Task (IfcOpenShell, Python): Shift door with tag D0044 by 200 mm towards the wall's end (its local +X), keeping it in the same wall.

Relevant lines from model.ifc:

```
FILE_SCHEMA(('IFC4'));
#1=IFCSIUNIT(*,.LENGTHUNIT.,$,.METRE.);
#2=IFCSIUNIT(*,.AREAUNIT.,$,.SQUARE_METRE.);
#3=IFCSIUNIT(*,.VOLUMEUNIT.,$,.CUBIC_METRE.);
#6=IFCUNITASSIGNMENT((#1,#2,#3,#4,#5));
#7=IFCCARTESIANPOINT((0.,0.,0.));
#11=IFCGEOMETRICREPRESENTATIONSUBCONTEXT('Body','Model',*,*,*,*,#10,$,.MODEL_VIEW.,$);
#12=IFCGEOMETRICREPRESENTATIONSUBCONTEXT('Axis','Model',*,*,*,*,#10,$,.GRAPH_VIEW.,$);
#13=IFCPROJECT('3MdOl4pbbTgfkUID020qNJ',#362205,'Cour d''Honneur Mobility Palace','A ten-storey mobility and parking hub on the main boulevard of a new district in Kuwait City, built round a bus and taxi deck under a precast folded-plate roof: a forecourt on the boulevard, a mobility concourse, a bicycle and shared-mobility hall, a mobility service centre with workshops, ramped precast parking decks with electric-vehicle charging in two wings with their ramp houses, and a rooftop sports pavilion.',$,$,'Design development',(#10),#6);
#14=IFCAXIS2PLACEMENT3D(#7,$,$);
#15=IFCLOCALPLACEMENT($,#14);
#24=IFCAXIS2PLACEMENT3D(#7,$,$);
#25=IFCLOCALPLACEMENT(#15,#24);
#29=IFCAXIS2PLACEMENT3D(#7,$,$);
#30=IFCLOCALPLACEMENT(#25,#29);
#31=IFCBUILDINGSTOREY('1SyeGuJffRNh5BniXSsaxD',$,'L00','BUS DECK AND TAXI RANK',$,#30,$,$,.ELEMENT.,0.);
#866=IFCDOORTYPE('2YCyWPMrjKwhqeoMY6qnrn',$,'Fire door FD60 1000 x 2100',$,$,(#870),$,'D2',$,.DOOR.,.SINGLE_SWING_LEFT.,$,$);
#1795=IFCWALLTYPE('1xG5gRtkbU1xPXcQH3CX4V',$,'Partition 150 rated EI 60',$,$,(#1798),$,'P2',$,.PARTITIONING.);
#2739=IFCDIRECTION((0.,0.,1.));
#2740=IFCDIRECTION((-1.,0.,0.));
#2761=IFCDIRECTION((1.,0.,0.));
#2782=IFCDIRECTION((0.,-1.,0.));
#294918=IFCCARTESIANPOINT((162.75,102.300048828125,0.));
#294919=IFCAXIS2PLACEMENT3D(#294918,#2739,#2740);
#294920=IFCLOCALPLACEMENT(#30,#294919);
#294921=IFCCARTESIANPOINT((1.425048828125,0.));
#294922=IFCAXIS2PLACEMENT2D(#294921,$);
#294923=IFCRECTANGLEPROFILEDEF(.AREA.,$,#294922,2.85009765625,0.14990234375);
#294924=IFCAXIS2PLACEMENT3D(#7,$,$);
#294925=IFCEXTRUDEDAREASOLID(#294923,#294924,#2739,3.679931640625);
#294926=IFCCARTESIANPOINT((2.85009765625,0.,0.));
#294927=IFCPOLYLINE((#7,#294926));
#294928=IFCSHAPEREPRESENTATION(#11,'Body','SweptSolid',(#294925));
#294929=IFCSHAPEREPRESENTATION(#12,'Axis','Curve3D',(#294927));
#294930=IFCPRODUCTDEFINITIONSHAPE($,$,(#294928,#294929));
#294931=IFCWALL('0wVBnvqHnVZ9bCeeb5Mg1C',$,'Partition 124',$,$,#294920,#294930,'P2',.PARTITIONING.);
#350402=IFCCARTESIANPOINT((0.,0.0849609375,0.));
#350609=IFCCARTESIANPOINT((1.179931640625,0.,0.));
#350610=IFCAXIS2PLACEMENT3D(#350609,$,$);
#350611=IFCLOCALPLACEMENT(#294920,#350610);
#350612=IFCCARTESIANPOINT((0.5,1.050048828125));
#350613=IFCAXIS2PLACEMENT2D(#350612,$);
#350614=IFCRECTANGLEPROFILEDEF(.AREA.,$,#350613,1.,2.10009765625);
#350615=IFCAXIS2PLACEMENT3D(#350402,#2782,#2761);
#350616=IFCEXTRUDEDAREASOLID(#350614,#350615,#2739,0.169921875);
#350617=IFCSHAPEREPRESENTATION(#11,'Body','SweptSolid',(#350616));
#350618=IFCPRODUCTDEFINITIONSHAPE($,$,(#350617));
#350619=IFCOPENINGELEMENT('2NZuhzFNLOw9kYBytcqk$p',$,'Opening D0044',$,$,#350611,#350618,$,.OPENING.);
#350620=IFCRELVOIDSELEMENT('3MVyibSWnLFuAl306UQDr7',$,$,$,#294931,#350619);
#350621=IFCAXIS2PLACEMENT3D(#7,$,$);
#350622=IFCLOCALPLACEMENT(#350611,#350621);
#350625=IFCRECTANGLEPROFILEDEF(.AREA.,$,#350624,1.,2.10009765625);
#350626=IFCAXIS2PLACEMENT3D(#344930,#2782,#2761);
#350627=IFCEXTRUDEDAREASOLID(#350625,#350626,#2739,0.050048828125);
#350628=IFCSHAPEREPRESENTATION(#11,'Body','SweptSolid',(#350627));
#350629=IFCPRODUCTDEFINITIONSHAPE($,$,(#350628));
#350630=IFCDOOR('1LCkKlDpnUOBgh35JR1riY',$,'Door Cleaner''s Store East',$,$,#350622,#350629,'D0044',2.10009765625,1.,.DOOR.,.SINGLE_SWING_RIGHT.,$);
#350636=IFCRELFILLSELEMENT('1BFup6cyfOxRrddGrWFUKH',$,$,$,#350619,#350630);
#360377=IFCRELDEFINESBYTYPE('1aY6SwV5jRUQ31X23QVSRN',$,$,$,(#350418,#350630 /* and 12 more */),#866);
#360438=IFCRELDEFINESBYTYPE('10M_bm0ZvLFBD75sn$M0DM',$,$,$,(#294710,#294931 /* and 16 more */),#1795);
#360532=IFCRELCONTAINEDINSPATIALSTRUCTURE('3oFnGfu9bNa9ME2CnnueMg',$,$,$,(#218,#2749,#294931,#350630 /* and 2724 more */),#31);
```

```python
import ifcopenshell
import ifcopenshell.api.geometry
import ifcopenshell.util.placement
import ifcopenshell.util.unit

model = ifcopenshell.open("model.ifc")
unit_scale = ifcopenshell.util.unit.calculate_unit_scale(model)

door = model.by_guid("1LCkKlDpnUOBgh35JR1riY")
opening = door.FillsVoids[0].RelatingOpeningElement
wall = opening.VoidsElements[0].RelatingBuildingElement

wall_matrix = ifcopenshell.util.placement.get_local_placement(wall.ObjectPlacement)
shift = wall_matrix[:3, 0] * 0.2 / unit_scale
before = ifcopenshell.util.placement.get_local_placement(door.ObjectPlacement)[:3, 3].copy()

# The door is placed relative to its opening, so it follows when the opening moves.
matrix = ifcopenshell.util.placement.get_local_placement(opening.ObjectPlacement)
matrix[:3, 3] += shift
ifcopenshell.api.geometry.edit_object_placement(
    model, product=opening, matrix=matrix, is_si=False, should_transform_children=True
)

after = ifcopenshell.util.placement.get_local_placement(door.ObjectPlacement)[:3, 3]
print("door moved by", (after - before).round(3) + 0.0)

model.write("model_v2.ifc")
```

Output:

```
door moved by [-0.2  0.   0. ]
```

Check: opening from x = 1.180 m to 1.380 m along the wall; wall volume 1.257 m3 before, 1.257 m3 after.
